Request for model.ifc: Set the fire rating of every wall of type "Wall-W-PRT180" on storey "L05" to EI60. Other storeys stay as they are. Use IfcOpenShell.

First a look at what the model holds.

```python
import ifcopenshell
import ifcopenshell.util.element

model = ifcopenshell.open("model.ifc")
print(model.schema)
storey = next(s for s in model.by_type("IfcBuildingStorey") if s.Name == "L05")
walls = [e for e in ifcopenshell.util.element.get_decomposition(storey) if e.is_a("IfcWall")]
seen = {}
for e in walls:
    element_type = ifcopenshell.util.element.get_type(e)
    key = (element_type.Name if element_type != e and element_type else None, ifcopenshell.util.element.get_pset(e, "Pset_WallCommon", "FireRating"))
    seen[key] = seen.get(key, 0) + 1
for (name, value), count in sorted(seen.items(), key=str):
    print(count, "x", name, "|", value)
```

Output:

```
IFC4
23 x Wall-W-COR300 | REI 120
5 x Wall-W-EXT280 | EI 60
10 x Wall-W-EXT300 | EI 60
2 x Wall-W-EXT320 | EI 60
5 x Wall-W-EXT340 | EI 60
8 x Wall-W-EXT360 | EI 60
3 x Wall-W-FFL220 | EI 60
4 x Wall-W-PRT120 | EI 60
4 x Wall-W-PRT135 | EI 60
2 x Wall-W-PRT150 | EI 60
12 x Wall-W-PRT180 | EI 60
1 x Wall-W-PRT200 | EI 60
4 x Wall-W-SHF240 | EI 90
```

```python
import ifcopenshell
import ifcopenshell.api.pset
import ifcopenshell.util.element

model = ifcopenshell.open("model.ifc")

storey = next(s for s in model.by_type("IfcBuildingStorey") if s.Name == "L05")
walls = [e for e in ifcopenshell.util.element.get_decomposition(storey) if e.is_a("IfcWall")]

count = 0
for e in walls:
    element_type = ifcopenshell.util.element.get_type(e)
    if element_type in (None, e) or element_type.Name != "Wall-W-PRT180":
        continue
    # add_pset returns the element's existing set when there is one.
    pset = ifcopenshell.api.pset.add_pset(model, product=e, name="Pset_WallCommon")
    ifcopenshell.api.pset.edit_pset(model, pset=pset, properties={"FireRating": "EI60"})
    count += 1

print(count, "walls updated")

model.write("model_rev.ifc")
```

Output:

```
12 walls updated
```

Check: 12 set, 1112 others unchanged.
